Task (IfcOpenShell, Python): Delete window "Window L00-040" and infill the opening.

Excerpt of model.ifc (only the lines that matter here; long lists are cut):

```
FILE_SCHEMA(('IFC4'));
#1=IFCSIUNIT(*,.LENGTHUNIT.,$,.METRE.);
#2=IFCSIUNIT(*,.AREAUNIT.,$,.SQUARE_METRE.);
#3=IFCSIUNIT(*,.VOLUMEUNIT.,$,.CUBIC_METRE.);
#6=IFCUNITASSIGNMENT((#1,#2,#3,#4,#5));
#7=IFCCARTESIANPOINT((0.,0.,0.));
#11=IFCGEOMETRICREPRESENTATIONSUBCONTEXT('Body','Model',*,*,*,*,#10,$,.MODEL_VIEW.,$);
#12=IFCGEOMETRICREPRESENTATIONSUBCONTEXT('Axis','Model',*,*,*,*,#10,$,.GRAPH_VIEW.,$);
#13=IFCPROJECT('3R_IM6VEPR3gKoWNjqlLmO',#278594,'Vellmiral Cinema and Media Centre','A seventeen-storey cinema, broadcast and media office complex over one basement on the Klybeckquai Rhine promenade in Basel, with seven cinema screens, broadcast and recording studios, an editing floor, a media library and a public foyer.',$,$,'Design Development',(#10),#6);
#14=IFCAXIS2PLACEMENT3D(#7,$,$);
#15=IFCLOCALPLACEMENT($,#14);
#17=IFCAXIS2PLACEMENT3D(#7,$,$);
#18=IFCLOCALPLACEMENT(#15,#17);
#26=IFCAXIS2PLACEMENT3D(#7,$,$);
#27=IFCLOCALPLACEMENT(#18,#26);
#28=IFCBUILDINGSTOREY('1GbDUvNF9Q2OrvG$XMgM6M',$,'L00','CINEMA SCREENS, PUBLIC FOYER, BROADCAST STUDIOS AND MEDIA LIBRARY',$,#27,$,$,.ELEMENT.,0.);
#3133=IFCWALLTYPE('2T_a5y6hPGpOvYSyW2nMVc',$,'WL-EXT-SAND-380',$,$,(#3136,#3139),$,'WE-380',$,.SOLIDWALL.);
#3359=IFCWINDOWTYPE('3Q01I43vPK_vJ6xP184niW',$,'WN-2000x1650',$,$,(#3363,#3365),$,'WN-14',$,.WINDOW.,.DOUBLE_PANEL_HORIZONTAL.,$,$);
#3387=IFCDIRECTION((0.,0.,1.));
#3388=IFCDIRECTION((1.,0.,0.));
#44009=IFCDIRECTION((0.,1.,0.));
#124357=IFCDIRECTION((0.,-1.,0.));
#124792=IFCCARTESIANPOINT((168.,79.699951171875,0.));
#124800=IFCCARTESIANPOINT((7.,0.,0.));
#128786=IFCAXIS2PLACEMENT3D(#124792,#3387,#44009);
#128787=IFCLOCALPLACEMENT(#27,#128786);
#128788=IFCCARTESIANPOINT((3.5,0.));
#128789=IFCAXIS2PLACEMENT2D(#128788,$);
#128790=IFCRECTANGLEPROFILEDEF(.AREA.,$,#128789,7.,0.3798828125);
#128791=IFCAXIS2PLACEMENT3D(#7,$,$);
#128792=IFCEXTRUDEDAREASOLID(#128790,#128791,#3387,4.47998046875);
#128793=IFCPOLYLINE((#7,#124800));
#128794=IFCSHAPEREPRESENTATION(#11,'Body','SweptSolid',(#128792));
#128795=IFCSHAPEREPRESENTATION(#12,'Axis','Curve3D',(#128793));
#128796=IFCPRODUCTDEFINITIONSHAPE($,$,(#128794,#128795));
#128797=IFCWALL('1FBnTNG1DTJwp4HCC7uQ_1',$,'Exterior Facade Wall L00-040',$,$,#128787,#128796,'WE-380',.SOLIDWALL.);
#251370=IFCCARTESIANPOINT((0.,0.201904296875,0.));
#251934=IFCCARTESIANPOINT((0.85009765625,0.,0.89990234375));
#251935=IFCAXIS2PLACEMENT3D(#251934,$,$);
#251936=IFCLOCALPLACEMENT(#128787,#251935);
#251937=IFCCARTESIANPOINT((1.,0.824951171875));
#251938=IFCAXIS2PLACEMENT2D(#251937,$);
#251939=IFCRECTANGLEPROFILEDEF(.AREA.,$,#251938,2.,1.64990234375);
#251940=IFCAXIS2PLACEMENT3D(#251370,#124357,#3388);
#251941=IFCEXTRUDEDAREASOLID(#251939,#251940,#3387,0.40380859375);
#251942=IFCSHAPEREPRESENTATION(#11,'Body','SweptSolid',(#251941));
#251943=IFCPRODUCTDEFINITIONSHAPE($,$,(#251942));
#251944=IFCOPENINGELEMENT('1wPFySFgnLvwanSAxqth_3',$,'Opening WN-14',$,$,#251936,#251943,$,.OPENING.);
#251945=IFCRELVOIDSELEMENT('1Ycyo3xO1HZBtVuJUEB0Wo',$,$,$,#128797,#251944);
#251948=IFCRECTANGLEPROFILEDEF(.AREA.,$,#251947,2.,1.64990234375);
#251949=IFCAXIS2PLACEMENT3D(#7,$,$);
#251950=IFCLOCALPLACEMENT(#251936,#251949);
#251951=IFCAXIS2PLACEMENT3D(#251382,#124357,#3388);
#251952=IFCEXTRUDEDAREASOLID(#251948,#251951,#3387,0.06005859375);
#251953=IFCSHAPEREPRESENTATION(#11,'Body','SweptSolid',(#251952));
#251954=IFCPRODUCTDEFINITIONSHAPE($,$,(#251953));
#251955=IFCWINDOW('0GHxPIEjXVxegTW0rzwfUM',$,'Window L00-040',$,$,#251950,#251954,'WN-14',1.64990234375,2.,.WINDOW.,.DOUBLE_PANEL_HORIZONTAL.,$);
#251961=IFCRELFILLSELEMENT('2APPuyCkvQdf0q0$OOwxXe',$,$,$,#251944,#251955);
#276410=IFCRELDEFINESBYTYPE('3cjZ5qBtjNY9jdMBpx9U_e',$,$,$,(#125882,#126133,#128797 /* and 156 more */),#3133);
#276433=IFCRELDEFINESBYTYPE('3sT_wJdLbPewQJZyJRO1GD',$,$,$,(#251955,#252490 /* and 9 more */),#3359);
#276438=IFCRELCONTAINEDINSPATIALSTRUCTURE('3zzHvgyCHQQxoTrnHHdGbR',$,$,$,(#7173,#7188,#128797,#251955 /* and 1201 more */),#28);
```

```python
import ifcopenshell
import ifcopenshell.api.feature
import ifcopenshell.api.root
import ifcopenshell.geom
import ifcopenshell.util.shape

model = ifcopenshell.open("model.ifc")
settings = ifcopenshell.geom.settings()


def volume(element):
    """Net volume in cubic metres, openings subtracted."""
    shape = ifcopenshell.geom.create_shape(settings, element)
    return ifcopenshell.util.shape.get_volume(shape.geometry)


window = model.by_guid("0GHxPIEjXVxegTW0rzwfUM")
opening = window.FillsVoids[0].RelatingOpeningElement
wall = opening.VoidsElements[0].RelatingBuildingElement
before = volume(wall)

ifcopenshell.api.root.remove_product(model, product=window)
ifcopenshell.api.feature.remove_feature(model, feature=opening)

after = volume(wall)

print(f"wall volume {before:.3f} -> {after:.3f} m3")

model.write("model_rev.ifc")
```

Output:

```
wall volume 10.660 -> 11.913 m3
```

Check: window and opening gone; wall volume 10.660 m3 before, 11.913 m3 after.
